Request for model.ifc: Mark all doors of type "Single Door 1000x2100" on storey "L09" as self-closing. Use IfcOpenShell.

First a look at what the model holds.

```python
import ifcopenshell
import ifcopenshell.util.element

model = ifcopenshell.open("model.ifc")
print(model.schema)
storey = next(s for s in model.by_type("IfcBuildingStorey") if s.Name == "L09")
doors = [e for e in ifcopenshell.util.element.get_decomposition(storey) if e.is_a("IfcDoor")]
seen = {}
for e in doors:
    element_type = ifcopenshell.util.element.get_type(e)
    key = (element_type.Name if element_type != e and element_type else None, ifcopenshell.util.element.get_pset(e, "Pset_DoorCommon", "SelfClosing"))
    seen[key] = seen.get(key, 0) + 1
for (name, value), count in sorted(seen.items(), key=str):
    print(count, "x", name, "|", value)
```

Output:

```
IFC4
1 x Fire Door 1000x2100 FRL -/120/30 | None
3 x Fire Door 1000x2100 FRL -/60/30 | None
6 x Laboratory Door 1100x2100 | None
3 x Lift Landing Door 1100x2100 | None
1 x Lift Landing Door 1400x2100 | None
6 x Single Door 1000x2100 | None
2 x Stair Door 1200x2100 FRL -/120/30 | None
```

```python
import ifcopenshell
import ifcopenshell.api.pset
import ifcopenshell.util.element

model = ifcopenshell.open("model.ifc")

storey = next(s for s in model.by_type("IfcBuildingStorey") if s.Name == "L09")
doors = [e for e in ifcopenshell.util.element.get_decomposition(storey) if e.is_a("IfcDoor")]

count = 0
for e in doors:
    element_type = ifcopenshell.util.element.get_type(e)
    if element_type in (None, e) or element_type.Name != "Single Door 1000x2100":
        continue
    # add_pset returns the element's existing set when there is one.
    pset = ifcopenshell.api.pset.add_pset(model, product=e, name="Pset_DoorCommon")
    ifcopenshell.api.pset.edit_pset(model, pset=pset, properties={"SelfClosing": True})
    count += 1

print(count, "doors updated")

model.write("model_rev.ifc")
```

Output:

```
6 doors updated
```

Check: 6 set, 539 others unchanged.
